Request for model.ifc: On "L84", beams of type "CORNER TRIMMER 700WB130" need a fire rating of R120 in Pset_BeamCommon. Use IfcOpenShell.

First a look at what the model holds.

```python
import ifcopenshell
import ifcopenshell.util.element

model = ifcopenshell.open("model.ifc")
print(model.schema)
storey = next(s for s in model.by_type("IfcBuildingStorey") if s.Name == "L84")
beams = [e for e in ifcopenshell.util.element.get_decomposition(storey) if e.is_a("IfcBeam")]
seen = {}
for e in beams:
    element_type = ifcopenshell.util.element.get_type(e)
    key = (element_type.Name if element_type != e and element_type else None, ifcopenshell.util.element.get_pset(e, "Pset_BeamCommon", "FireRating"))
    seen[key] = seen.get(key, 0) + 1
for (name, value), count in sorted(seen.items(), key=str):
    print(count, "x", name, "|", value)
```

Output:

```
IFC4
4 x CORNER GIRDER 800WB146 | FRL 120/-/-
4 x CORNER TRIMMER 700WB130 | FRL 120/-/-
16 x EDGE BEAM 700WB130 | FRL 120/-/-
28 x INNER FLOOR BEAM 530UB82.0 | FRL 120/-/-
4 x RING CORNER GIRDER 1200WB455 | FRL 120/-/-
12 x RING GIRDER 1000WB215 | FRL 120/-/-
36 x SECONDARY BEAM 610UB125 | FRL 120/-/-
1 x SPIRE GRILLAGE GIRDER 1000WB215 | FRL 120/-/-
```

```python
import ifcopenshell
import ifcopenshell.api.pset
import ifcopenshell.util.element

model = ifcopenshell.open("model.ifc")

storey = next(s for s in model.by_type("IfcBuildingStorey") if s.Name == "L84")
beams = [e for e in ifcopenshell.util.element.get_decomposition(storey) if e.is_a("IfcBeam")]

count = 0
for e in beams:
    element_type = ifcopenshell.util.element.get_type(e)
    if element_type in (None, e) or element_type.Name != "CORNER TRIMMER 700WB130":
        continue
    found = ifcopenshell.util.element.get_pset(e, "Pset_BeamCommon", should_inherit=False)
    if found:
        pset = model.by_id(found["id"])
        if len(ifcopenshell.util.element.get_elements_by_pset(pset)) > 1:
            pset = ifcopenshell.api.pset.unshare_pset(model, products=[e], pset=pset)[0]
    else:
        pset = ifcopenshell.api.pset.add_pset(model, product=e, name="Pset_BeamCommon")
    ifcopenshell.api.pset.edit_pset(model, pset=pset, properties={"FireRating": "R120"})
    count += 1

print(count, "beams updated")

model.write("model_v2.ifc")
```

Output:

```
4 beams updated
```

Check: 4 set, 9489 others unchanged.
